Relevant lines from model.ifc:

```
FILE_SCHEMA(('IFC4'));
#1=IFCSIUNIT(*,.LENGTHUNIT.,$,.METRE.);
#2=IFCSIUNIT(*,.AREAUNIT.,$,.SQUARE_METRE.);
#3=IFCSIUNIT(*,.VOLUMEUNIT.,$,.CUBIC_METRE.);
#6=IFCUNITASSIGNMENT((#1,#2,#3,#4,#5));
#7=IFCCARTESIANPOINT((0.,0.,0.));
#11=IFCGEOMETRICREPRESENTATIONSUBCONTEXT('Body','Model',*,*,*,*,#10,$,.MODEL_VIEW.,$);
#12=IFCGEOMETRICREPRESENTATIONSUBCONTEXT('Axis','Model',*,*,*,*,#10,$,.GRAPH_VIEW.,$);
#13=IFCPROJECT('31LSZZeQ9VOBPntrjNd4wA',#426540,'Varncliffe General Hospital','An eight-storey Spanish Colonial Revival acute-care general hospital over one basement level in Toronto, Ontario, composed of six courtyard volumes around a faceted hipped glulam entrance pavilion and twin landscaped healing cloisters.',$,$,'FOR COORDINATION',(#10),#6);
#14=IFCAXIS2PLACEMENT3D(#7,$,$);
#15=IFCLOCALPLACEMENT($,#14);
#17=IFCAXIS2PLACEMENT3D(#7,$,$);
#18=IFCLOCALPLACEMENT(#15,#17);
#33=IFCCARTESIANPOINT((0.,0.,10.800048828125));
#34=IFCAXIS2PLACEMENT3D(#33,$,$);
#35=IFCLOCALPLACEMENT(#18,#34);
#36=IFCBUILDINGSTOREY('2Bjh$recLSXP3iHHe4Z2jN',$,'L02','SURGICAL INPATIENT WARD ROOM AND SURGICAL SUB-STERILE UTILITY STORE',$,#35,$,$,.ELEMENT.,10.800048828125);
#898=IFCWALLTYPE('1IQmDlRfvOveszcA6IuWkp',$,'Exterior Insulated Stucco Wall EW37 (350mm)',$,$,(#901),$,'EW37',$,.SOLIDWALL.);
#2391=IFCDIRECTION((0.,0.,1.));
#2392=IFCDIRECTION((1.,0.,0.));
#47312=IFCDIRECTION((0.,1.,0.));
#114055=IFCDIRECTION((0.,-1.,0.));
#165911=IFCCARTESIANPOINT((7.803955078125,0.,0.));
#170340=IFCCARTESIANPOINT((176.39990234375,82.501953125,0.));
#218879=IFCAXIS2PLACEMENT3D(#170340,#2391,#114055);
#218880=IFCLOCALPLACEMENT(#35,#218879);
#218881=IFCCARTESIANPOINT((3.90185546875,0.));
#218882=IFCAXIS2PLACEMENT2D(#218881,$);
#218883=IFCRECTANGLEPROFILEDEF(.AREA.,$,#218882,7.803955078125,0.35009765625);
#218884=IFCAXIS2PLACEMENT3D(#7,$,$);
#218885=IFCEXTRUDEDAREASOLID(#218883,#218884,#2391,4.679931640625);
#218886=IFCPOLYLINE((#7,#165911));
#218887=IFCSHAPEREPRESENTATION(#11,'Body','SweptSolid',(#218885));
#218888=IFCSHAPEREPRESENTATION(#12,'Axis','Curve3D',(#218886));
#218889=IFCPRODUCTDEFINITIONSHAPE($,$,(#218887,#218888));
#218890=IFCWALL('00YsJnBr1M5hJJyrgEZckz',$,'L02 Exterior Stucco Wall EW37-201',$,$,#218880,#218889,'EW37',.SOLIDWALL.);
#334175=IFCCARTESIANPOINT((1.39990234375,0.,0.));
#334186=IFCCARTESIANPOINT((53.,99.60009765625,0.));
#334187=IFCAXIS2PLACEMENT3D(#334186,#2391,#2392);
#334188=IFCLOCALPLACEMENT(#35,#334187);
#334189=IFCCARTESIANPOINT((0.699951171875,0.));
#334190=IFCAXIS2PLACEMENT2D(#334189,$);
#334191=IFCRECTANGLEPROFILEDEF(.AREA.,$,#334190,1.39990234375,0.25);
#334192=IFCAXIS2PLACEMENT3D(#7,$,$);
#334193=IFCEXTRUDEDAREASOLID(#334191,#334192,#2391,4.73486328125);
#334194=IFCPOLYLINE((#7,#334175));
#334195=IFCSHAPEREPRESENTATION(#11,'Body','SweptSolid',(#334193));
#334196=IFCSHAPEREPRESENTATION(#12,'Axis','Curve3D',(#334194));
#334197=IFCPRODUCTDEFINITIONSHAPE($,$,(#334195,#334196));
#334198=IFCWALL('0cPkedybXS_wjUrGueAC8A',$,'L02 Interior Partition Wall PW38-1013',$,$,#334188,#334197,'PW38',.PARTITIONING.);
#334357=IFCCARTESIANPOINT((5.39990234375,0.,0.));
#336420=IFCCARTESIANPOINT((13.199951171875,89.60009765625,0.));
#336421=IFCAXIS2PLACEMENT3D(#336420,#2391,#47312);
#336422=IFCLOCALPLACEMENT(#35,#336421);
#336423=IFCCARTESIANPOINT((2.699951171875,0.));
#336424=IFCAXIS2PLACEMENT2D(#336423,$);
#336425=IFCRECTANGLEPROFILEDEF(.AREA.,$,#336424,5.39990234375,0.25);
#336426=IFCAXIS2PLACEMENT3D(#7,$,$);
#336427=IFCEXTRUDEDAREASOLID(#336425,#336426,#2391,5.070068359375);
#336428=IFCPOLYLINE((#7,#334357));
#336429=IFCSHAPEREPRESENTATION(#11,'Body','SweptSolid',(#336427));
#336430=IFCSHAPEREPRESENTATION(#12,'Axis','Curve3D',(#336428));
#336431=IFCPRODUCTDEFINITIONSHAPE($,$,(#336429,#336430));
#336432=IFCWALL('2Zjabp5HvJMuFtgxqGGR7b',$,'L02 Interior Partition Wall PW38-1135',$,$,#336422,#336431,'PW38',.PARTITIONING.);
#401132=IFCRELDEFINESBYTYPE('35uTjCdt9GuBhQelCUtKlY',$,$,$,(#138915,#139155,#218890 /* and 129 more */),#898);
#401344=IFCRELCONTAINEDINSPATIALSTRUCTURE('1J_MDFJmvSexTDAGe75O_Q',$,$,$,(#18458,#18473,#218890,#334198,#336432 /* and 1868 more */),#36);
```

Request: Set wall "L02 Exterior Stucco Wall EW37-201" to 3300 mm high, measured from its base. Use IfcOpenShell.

```python
import ifcopenshell
import ifcopenshell.geom
import ifcopenshell.util.representation
import ifcopenshell.util.shape
import ifcopenshell.util.unit

model = ifcopenshell.open("model.ifc")
unit_scale = ifcopenshell.util.unit.calculate_unit_scale(model)
settings = ifcopenshell.geom.settings()


def volume(element):
    """Net volume in cubic metres, openings subtracted."""
    shape = ifcopenshell.geom.create_shape(settings, element)
    return ifcopenshell.util.shape.get_volume(shape.geometry)


wall = model.by_id(218890)
before = volume(wall)

body = ifcopenshell.util.representation.get_representation(wall, "Model", "Body")
solid = body.Items[0]
old_height = solid.Depth
solid.Depth = 3.3 / unit_scale
after = volume(wall)

print(f"height {old_height:g} -> {solid.Depth:g}, volume {before:.3f} -> {after:.3f} m3")

model.write("model_edited.ifc")
```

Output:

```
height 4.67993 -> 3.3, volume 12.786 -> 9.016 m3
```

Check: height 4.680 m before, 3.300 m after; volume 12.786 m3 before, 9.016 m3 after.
